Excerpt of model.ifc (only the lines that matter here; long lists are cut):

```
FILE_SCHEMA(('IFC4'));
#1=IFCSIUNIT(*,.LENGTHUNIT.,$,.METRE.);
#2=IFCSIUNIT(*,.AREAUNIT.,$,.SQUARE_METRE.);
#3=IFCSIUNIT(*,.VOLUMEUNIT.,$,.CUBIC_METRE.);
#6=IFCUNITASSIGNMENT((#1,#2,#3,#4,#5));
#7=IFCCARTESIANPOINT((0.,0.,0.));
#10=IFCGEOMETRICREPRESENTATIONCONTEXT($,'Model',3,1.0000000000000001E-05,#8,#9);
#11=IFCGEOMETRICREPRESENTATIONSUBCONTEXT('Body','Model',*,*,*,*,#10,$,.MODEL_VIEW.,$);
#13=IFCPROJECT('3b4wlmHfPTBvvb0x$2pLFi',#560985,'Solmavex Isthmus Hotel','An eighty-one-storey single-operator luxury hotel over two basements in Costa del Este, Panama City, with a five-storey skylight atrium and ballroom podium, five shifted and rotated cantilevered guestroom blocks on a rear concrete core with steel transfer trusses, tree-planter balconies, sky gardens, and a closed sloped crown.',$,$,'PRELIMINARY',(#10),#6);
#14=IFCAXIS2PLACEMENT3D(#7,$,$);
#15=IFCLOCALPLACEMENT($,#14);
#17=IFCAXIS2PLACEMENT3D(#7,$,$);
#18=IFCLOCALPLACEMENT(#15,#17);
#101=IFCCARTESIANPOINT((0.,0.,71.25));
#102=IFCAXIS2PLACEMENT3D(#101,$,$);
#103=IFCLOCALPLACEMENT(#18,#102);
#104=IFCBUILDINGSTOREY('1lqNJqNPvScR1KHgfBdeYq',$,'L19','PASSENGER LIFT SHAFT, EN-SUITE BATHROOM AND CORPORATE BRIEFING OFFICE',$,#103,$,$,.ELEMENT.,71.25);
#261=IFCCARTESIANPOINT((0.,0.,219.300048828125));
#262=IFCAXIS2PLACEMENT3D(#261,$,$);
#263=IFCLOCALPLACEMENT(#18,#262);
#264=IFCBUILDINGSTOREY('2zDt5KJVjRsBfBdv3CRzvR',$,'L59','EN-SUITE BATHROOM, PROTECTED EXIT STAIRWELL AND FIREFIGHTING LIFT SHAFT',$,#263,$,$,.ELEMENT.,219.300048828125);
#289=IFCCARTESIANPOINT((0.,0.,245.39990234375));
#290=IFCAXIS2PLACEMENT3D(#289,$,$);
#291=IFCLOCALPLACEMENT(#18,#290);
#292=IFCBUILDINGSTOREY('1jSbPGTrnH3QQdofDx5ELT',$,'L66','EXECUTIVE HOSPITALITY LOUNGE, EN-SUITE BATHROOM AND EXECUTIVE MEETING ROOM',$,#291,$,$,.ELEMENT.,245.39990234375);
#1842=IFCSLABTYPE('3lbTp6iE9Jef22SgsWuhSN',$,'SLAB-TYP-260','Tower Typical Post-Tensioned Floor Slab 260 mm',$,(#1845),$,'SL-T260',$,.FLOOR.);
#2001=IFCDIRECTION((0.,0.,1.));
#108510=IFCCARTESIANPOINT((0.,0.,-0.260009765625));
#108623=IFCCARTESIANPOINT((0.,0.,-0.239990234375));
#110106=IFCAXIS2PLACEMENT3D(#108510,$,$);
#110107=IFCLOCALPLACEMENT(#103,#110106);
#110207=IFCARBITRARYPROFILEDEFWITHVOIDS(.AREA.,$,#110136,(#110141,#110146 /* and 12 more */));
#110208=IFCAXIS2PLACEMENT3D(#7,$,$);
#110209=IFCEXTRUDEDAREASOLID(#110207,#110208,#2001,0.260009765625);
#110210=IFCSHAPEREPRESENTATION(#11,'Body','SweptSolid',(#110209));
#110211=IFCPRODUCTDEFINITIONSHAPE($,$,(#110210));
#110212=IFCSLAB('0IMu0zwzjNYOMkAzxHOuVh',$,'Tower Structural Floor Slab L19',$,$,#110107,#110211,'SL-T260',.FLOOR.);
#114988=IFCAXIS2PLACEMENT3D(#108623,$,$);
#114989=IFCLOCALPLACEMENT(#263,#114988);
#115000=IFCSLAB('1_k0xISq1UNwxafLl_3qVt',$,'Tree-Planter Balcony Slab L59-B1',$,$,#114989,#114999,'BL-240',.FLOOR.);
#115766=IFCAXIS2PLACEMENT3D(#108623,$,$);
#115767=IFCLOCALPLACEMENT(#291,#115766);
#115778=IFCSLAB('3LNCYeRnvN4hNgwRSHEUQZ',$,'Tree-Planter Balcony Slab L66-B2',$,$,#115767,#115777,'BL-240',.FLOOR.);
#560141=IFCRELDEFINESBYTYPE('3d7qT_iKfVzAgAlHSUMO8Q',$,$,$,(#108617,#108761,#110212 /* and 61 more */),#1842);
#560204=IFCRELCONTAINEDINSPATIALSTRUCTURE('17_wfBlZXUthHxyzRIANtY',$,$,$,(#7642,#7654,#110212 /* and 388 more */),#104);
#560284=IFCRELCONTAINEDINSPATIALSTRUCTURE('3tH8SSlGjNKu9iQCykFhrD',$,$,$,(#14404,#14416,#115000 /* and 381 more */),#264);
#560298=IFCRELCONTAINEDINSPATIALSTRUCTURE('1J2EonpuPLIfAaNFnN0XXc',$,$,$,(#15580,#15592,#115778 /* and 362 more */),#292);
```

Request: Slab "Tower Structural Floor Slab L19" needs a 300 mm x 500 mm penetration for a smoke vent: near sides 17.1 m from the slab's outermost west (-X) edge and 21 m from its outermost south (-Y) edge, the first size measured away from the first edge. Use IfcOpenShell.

```python
import numpy as np
import ifcopenshell
import ifcopenshell.api.feature
import ifcopenshell.api.geometry
import ifcopenshell.api.root
import ifcopenshell.geom
import ifcopenshell.util.placement
import ifcopenshell.util.representation
import ifcopenshell.util.shape
import ifcopenshell.util.unit

model = ifcopenshell.open("model.ifc")
unit_scale = ifcopenshell.util.unit.calculate_unit_scale(model)
settings = ifcopenshell.geom.settings()


def volume(element):
    """Net volume in cubic metres, openings subtracted."""
    shape = ifcopenshell.geom.create_shape(settings, element)
    return ifcopenshell.util.shape.get_volume(shape.geometry)


slab = model.by_id(110212)
before = volume(slab)

# Extent in the slab's own axes, in metres. The edges named are its -X and -Y sides.
slab_shape = ifcopenshell.geom.create_shape(settings, slab)
vertices = ifcopenshell.util.shape.get_vertices(slab_shape.geometry)
x_min, y_min, bottom = vertices.min(axis=0)
top = vertices[:, 2].max()

opening = ifcopenshell.api.root.create_entity(model, ifc_class="IfcOpeningElement", name="Smoke vent opening", predefined_type="OPENING")
context = ifcopenshell.util.representation.get_context(model, "Model", "Body", "MODEL_VIEW")
width, depth = 0.3, 0.5
outline = [(0.0, 0.0), (width, 0.0), (width, depth), (0.0, depth), (0.0, 0.0)]
# Overshoot both faces by 50 mm so the cut is clean.
shape = ifcopenshell.api.geometry.add_slab_representation(
    model, context=context, depth=top - bottom + 0.1, polyline=outline
)
ifcopenshell.api.geometry.assign_representation(model, product=opening, representation=shape)

matrix = ifcopenshell.util.placement.get_local_placement(slab.ObjectPlacement)
matrix[:, 3] = matrix @ np.append(np.array([x_min + 17.1, y_min + 21, bottom - 0.05]) / unit_scale, 1.0)
ifcopenshell.api.geometry.edit_object_placement(model, product=opening, matrix=matrix, is_si=False)
ifcopenshell.api.feature.add_feature(model, feature=opening, element=slab)

after = volume(slab)

print(f"slab volume {before:.3f} -> {after:.3f} m3")

model.write("model-out.ifc")
```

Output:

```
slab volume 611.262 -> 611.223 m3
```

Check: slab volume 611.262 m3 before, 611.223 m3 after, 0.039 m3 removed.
